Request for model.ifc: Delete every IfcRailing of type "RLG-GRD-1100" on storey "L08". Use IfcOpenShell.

First a look at what the model holds.

```python
import ifcopenshell
import ifcopenshell.util.element

model = ifcopenshell.open("model.ifc")
print(model.schema)
storey = next(s for s in model.by_type("IfcBuildingStorey") if s.Name == "L08")
railings = [e for e in ifcopenshell.util.element.get_decomposition(storey) if e.is_a("IfcRailing")]
seen = {}
for e in railings:
    element_type = ifcopenshell.util.element.get_type(e)
    name = element_type.Name if element_type not in (None, e) else None
    seen[name] = seen.get(name, 0) + 1
for name, count in sorted(seen.items(), key=str):
    print(count, "x", name)
```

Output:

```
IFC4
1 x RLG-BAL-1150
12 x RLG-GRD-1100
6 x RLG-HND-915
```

```python
import ifcopenshell
import ifcopenshell.api.root
import ifcopenshell.util.element

model = ifcopenshell.open("model.ifc")

storey = next(s for s in model.by_type("IfcBuildingStorey") if s.Name == "L08")
railings = [e for e in ifcopenshell.util.element.get_decomposition(storey) if e.is_a("IfcRailing")]
targets = [e for e in railings if (t := ifcopenshell.util.element.get_type(e)) not in (None, e) and t.Name == "RLG-GRD-1100"]

for e in targets:
    ifcopenshell.api.root.remove_product(model, product=e)
print(len(targets), "removed")

model.write("model-out.ifc")
```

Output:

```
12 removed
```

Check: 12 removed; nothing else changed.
